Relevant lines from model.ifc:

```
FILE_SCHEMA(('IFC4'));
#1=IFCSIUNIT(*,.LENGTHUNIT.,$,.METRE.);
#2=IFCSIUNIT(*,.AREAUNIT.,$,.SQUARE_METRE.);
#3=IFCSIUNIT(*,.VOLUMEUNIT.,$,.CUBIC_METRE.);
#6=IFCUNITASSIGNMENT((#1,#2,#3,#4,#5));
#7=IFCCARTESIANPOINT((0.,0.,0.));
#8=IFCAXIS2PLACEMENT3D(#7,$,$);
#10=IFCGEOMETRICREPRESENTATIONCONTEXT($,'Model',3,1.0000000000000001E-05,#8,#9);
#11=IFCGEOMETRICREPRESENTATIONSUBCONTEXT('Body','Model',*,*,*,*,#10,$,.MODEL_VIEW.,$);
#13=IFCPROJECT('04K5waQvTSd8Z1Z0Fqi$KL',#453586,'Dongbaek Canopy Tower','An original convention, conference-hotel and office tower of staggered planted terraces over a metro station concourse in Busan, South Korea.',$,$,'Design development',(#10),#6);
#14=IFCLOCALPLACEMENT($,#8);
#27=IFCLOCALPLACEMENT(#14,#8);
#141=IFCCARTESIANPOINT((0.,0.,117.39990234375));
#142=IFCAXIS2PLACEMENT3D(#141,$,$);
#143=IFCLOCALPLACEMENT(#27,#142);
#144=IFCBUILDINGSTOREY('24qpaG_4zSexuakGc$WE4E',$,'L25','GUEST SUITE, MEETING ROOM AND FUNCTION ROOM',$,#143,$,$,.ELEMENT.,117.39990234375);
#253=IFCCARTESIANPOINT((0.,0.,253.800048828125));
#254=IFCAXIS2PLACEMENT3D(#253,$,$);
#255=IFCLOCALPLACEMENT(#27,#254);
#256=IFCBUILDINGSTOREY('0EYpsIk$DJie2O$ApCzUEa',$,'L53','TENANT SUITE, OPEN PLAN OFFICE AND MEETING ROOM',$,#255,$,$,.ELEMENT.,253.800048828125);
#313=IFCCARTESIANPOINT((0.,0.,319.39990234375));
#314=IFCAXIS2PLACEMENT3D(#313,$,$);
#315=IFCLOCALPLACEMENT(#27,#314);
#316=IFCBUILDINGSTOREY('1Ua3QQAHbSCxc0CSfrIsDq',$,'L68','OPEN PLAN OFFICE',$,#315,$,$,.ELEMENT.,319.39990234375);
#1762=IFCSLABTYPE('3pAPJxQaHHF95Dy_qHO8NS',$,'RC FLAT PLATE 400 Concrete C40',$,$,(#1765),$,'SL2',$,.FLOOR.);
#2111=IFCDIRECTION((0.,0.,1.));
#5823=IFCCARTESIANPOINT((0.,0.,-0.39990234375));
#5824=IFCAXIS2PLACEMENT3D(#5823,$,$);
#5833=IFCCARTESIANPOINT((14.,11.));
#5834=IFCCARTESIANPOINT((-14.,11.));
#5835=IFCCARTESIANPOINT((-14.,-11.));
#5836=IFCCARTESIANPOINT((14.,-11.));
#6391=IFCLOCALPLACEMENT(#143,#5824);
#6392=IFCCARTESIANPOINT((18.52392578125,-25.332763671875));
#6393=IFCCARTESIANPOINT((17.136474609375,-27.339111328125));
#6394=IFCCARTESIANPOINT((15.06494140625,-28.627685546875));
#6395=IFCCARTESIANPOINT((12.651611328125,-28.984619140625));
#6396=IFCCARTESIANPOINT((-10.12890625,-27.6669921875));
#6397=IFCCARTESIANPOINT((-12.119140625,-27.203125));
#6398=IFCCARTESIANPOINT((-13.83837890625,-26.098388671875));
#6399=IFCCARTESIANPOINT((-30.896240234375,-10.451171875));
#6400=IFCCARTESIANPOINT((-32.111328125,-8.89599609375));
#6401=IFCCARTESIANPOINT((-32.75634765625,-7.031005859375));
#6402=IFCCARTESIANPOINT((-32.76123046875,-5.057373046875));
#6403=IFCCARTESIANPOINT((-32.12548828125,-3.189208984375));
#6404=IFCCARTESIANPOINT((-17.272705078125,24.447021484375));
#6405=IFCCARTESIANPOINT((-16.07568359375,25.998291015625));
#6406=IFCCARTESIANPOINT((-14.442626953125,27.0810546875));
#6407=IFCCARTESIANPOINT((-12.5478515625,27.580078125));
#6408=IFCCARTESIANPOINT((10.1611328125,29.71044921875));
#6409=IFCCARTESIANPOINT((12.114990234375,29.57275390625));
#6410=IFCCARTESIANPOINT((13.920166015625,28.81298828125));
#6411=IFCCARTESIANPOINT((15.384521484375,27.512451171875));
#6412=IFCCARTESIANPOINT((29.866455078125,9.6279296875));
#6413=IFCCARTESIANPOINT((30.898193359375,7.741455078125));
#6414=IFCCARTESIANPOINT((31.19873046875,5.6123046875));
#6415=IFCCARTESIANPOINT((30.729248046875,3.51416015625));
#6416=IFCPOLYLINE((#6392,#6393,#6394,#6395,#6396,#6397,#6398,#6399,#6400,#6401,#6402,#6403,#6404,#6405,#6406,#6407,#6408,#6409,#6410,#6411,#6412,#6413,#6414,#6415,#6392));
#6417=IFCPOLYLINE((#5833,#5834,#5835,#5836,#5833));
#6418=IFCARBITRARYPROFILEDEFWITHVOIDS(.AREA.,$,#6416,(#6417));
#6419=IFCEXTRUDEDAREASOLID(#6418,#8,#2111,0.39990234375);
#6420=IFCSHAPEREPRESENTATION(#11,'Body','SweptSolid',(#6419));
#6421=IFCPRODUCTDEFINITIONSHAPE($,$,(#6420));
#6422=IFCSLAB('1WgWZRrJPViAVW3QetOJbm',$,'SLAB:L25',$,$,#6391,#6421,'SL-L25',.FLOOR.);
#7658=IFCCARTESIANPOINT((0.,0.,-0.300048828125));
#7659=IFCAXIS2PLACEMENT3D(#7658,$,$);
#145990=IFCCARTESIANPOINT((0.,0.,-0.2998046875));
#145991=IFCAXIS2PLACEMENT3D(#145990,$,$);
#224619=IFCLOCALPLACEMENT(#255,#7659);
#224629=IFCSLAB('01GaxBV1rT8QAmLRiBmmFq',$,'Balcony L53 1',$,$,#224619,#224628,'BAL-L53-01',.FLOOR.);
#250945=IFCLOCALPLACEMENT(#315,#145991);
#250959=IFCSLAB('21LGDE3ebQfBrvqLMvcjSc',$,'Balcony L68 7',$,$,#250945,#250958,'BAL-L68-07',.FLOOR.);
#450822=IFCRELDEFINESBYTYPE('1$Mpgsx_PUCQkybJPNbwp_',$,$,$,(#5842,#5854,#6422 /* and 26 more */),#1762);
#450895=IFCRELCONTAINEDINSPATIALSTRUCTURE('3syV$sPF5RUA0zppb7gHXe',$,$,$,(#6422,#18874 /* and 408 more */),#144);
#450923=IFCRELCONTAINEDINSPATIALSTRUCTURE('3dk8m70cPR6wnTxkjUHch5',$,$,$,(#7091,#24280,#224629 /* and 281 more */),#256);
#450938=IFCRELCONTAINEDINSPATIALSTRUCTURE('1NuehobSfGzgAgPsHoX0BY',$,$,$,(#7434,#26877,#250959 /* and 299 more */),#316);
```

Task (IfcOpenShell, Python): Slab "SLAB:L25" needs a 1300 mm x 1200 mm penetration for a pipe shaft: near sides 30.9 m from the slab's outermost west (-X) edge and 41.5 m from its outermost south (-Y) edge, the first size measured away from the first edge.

```python
import numpy as np
import ifcopenshell
import ifcopenshell.api.feature
import ifcopenshell.api.geometry
import ifcopenshell.api.root
import ifcopenshell.geom
import ifcopenshell.util.placement
import ifcopenshell.util.representation
import ifcopenshell.util.shape
import ifcopenshell.util.unit

model = ifcopenshell.open("model.ifc")
unit_scale = ifcopenshell.util.unit.calculate_unit_scale(model)
settings = ifcopenshell.geom.settings()


def volume(element):
    """Net volume in cubic metres, openings subtracted."""
    shape = ifcopenshell.geom.create_shape(settings, element)
    return ifcopenshell.util.shape.get_volume(shape.geometry)


slab = model.by_id(6422)
before = volume(slab)

# Extent in the slab's own axes, in metres. The edges named are its -X and -Y sides.
slab_shape = ifcopenshell.geom.create_shape(settings, slab)
vertices = ifcopenshell.util.shape.get_vertices(slab_shape.geometry)
x_min, y_min, bottom = vertices.min(axis=0)
top = vertices[:, 2].max()

opening = ifcopenshell.api.root.create_entity(model, ifc_class="IfcOpeningElement", name="Pipe shaft opening", predefined_type="OPENING")
context = ifcopenshell.util.representation.get_context(model, "Model", "Body", "MODEL_VIEW")
width, depth = 1.3, 1.2
outline = [(0.0, 0.0), (width, 0.0), (width, depth), (0.0, depth), (0.0, 0.0)]
# Overshoot both faces by 50 mm so the cut is clean.
shape = ifcopenshell.api.geometry.add_slab_representation(
    model, context=context, depth=top - bottom + 0.1, polyline=outline
)
ifcopenshell.api.geometry.assign_representation(model, product=opening, representation=shape)

matrix = ifcopenshell.util.placement.get_local_placement(slab.ObjectPlacement)
matrix[:, 3] = matrix @ np.append(np.array([x_min + 30.9, y_min + 41.5, bottom - 0.05]) / unit_scale, 1.0)
ifcopenshell.api.geometry.edit_object_placement(model, product=opening, matrix=matrix, is_si=False)
ifcopenshell.api.feature.add_feature(model, feature=opening, element=slab)

after = volume(slab)

print(f"slab volume {before:.3f} -> {after:.3f} m3")

model.write("model_v2.ifc")
```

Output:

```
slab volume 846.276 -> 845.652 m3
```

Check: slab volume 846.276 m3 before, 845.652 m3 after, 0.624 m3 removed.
